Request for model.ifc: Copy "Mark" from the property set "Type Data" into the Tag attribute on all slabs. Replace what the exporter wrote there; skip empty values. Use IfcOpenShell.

First a look at what the model holds.

```python
import ifcopenshell
import ifcopenshell.util.element

model = ifcopenshell.open("model.ifc")
print(model.schema)
slabs = model.by_type("IfcSlab")
print(len(slabs), "slabs")
for e in slabs[:8]:
    source = ifcopenshell.util.element.get_pset(e, "Type Data", "Mark")
    target = e.Tag
    print(e.id(), repr(source), repr(target), sep=" | ")
```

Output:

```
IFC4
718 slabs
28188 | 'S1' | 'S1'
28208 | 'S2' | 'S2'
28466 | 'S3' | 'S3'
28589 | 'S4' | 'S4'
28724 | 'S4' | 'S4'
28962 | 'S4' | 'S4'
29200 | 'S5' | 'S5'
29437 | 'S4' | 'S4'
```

```python
import ifcopenshell
import ifcopenshell.util.element

model = ifcopenshell.open("model.ifc")

count = 0
for e in model.by_type("IfcSlab"):
    value = ifcopenshell.util.element.get_pset(e, "Type Data", "Mark")
    current = e.Tag
    if not value or not value.strip() or current == value:
        continue
    e.Tag = value
    count += 1

print(count, "slabs updated")

model.write("model_rev.ifc")
```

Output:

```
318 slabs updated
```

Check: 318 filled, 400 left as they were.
